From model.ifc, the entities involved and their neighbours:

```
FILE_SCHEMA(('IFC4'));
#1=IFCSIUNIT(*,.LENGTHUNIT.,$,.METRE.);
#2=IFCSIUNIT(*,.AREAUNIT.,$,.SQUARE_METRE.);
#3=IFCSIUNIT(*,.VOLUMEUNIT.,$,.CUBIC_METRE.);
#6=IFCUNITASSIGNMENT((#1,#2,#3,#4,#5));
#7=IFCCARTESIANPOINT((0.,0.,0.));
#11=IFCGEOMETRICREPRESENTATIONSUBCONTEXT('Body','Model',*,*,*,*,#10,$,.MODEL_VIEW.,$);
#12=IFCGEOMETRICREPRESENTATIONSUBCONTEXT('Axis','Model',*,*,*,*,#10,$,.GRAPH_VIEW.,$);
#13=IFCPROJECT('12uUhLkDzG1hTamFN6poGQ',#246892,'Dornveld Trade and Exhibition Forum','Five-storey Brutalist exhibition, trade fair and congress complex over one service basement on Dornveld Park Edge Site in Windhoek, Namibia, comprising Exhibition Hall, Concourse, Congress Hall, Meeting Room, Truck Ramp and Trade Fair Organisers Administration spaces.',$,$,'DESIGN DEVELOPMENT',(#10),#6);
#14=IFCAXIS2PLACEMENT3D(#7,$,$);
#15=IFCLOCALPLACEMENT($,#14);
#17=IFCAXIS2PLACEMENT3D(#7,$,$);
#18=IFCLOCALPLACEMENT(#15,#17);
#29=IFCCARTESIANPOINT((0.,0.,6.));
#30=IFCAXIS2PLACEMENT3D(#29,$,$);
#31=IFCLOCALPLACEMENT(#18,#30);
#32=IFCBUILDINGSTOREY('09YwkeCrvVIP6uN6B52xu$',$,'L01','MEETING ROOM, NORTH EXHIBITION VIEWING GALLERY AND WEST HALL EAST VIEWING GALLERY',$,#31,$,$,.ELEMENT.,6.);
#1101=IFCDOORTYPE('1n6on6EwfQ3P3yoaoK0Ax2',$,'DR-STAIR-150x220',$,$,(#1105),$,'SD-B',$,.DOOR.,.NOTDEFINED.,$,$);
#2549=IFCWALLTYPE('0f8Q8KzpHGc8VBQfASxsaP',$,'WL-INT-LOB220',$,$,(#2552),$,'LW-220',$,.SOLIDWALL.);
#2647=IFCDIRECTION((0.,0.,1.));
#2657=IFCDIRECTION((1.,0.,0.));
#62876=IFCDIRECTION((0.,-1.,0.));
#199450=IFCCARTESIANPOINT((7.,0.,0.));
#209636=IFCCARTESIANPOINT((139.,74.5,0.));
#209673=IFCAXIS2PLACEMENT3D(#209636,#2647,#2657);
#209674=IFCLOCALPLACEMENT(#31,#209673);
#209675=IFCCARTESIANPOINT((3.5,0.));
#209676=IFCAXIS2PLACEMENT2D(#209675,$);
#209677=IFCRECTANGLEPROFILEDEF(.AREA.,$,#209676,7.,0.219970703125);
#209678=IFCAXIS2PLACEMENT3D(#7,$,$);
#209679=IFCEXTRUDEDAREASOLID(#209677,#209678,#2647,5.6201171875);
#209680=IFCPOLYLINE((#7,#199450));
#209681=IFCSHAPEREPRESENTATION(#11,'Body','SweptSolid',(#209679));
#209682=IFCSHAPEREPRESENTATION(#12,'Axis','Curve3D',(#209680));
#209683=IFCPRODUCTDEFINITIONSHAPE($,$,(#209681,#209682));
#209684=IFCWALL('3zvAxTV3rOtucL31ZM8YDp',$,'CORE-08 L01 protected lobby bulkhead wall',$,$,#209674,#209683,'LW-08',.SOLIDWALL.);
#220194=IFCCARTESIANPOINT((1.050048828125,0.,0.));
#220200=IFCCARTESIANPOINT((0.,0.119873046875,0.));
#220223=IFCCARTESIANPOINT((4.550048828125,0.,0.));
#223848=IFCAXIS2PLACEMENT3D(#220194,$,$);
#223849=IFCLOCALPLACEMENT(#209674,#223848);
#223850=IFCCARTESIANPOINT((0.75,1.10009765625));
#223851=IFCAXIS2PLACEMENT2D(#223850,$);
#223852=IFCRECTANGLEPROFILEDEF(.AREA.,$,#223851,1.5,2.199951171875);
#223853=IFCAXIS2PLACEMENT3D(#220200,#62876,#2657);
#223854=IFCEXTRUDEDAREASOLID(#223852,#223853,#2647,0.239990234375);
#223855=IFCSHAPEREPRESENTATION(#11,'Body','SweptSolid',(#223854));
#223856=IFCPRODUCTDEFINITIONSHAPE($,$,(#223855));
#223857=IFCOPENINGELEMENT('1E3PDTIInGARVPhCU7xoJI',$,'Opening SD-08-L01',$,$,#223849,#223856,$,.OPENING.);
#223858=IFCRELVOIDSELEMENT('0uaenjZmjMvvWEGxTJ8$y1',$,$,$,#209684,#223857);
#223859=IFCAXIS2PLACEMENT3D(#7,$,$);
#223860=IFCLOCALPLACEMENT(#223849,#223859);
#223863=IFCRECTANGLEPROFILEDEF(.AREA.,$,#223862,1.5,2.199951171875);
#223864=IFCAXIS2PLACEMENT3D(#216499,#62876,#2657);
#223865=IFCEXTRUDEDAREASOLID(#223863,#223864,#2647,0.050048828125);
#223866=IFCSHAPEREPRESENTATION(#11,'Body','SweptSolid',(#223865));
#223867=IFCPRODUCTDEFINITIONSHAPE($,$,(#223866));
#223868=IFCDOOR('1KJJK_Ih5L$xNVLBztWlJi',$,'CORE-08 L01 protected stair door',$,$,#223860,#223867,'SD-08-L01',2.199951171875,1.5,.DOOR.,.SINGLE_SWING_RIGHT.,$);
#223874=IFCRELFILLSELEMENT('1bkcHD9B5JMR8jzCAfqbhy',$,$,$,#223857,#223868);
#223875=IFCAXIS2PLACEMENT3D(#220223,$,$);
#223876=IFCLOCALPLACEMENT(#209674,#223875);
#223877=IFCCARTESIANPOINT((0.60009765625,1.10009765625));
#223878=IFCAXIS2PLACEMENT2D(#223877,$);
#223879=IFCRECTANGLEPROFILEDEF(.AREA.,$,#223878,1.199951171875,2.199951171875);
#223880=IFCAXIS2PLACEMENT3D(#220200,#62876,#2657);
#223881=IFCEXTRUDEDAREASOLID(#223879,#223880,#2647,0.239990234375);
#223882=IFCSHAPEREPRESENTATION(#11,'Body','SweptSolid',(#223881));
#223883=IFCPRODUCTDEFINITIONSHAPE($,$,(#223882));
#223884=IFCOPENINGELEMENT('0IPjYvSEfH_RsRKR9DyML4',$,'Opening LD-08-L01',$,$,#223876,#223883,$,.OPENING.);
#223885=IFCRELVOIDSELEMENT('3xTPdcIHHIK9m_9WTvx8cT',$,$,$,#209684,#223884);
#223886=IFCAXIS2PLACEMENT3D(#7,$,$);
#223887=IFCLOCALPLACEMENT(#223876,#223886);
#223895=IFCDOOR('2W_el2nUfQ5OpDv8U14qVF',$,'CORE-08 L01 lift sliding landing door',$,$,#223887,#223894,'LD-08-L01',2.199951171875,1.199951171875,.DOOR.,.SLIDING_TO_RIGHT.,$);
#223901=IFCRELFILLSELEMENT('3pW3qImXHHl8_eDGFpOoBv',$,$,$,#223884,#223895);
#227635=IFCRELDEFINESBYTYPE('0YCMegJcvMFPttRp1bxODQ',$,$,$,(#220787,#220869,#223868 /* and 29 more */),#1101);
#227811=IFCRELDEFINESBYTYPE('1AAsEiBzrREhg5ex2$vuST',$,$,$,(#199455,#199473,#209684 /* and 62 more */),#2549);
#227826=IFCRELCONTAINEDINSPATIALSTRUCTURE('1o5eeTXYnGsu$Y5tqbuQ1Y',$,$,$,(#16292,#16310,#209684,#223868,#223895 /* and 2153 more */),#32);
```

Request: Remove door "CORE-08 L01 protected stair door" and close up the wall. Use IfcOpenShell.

```python
import ifcopenshell
import ifcopenshell.api.feature
import ifcopenshell.api.root
import ifcopenshell.geom
import ifcopenshell.util.shape

model = ifcopenshell.open("model.ifc")
settings = ifcopenshell.geom.settings()


def volume(element):
    """Net volume in cubic metres, openings subtracted."""
    shape = ifcopenshell.geom.create_shape(settings, element)
    return ifcopenshell.util.shape.get_volume(shape.geometry)


door = model.by_guid("1KJJK_Ih5L$xNVLBztWlJi")
opening = door.FillsVoids[0].RelatingOpeningElement
wall = opening.VoidsElements[0].RelatingBuildingElement
before = volume(wall)

ifcopenshell.api.root.remove_product(model, product=door)
ifcopenshell.api.feature.remove_feature(model, feature=opening)

after = volume(wall)

print(f"wall volume {before:.3f} -> {after:.3f} m3")

model.write("model_rev.ifc")
```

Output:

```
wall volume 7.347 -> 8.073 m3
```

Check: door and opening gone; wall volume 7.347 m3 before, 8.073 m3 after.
